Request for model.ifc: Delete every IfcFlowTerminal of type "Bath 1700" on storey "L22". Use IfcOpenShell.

First a look at what the model holds.

```python
import ifcopenshell
import ifcopenshell.util.element

model = ifcopenshell.open("model.ifc")
print(model.schema)
storey = next(s for s in model.by_type("IfcBuildingStorey") if s.Name == "L22")
terminals = [e for e in ifcopenshell.util.element.get_decomposition(storey) if e.is_a("IfcFlowTerminal")]
seen = {}
for e in terminals:
    element_type = ifcopenshell.util.element.get_type(e)
    name = element_type.Name if element_type not in (None, e) else None
    seen[name] = seen.get(name, 0) + 1
for name, count in sorted(seen.items(), key=str):
    print(count, "x", name)
```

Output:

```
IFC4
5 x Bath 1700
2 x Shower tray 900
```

```python
import ifcopenshell
import ifcopenshell.api.root
import ifcopenshell.util.element

model = ifcopenshell.open("model.ifc")

storey = next(s for s in model.by_type("IfcBuildingStorey") if s.Name == "L22")
terminals = [e for e in ifcopenshell.util.element.get_decomposition(storey) if e.is_a("IfcFlowTerminal")]
targets = [e for e in terminals if (t := ifcopenshell.util.element.get_type(e)) not in (None, e) and t.Name == "Bath 1700"]

for e in targets:
    ifcopenshell.api.root.remove_product(model, product=e)
print(len(targets), "removed")

model.write("model_updated.ifc")
```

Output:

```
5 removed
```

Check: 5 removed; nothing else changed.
